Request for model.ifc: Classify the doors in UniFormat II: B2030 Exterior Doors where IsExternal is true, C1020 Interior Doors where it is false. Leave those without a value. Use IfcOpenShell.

First a look at what the model holds.

```python
import ifcopenshell
import ifcopenshell.util.element

model = ifcopenshell.open("model.ifc")
print(model.schema)
print("classifications:", [c.Name for c in model.by_type("IfcClassification")])
values = [ifcopenshell.util.element.get_pset(e, "Pset_DoorCommon", "IsExternal") for e in model.by_type("IfcDoor")]
for value in (True, False, None):
    print("IsExternal", value, values.count(value))
```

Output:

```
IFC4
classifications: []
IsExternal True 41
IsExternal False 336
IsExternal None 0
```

```python
import ifcopenshell
import ifcopenshell.api.classification
import ifcopenshell.util.element

model = ifcopenshell.open("model.ifc")

system = ifcopenshell.api.classification.add_classification(model, classification="UniFormat II")

doors = model.by_type("IfcDoor")
external = {e: ifcopenshell.util.element.get_pset(e, "Pset_DoorCommon", "IsExternal") for e in doors}
for flag, code, name in ((True, "B2030", "Exterior Doors"), (False, "C1020", "Interior Doors")):
    products = [e for e in doors if external[e] is flag]
    ifcopenshell.api.classification.add_reference(
        model, products=products, classification=system, identification=code, name=name
    )
    print(code, len(products))

model.write("model_updated.ifc")
```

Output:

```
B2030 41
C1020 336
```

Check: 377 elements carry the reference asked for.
